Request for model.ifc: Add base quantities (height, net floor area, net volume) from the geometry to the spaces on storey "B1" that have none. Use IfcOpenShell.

First a look at what the model holds.

```python
import ifcopenshell
import ifcopenshell.util.element
import ifcopenshell.util.unit

model = ifcopenshell.open("model.ifc")
print(model.schema)
for unit_type in ("LENGTHUNIT", "AREAUNIT", "VOLUMEUNIT"):
    print(unit_type, ifcopenshell.util.unit.calculate_unit_scale(model, unit_type))
storey = next(s for s in model.by_type("IfcBuildingStorey") if s.Name == "B1")
spaces = [e for e in ifcopenshell.util.element.get_decomposition(storey) if e.is_a("IfcSpace")]
for e in sorted(spaces, key=lambda e: e.id()):
    print(e.id(), e.is_a(), e.Name, list(ifcopenshell.util.element.get_psets(e, qtos_only=True)), sep=" | ")
```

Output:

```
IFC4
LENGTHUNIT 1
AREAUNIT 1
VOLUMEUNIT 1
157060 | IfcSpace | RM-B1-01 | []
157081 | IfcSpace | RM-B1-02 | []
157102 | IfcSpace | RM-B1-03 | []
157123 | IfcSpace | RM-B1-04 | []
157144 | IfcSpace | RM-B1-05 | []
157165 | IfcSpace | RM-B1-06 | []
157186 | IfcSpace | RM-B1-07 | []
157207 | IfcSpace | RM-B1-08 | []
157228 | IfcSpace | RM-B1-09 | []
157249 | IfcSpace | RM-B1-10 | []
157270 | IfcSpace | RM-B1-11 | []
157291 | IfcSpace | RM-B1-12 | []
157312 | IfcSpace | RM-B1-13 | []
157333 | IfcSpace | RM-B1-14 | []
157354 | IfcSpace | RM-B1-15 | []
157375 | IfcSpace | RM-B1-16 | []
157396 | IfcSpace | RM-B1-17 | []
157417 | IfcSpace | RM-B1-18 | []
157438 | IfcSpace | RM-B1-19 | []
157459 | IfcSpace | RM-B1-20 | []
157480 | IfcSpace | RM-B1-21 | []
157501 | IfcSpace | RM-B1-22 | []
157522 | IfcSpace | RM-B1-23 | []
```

```python
import ifcopenshell
import ifcopenshell.api.pset
import ifcopenshell.geom
import ifcopenshell.util.element
import ifcopenshell.util.shape
import ifcopenshell.util.unit

model = ifcopenshell.open("model.ifc")
unit_scale = ifcopenshell.util.unit.calculate_unit_scale(model)
area_scale = ifcopenshell.util.unit.calculate_unit_scale(model, "AREAUNIT")
volume_scale = ifcopenshell.util.unit.calculate_unit_scale(model, "VOLUMEUNIT")
settings = ifcopenshell.geom.settings()

storey = next(s for s in model.by_type("IfcBuildingStorey") if s.Name == "B1")
spaces = [e for e in ifcopenshell.util.element.get_decomposition(storey) if e.is_a("IfcSpace")]

for e in sorted(spaces, key=lambda e: e.id()):
    if ifcopenshell.util.element.get_psets(e, qtos_only=True, should_inherit=False):
        continue
    # Geometry comes back in metres, in the element's own axes.
    shape = ifcopenshell.geom.create_shape(settings, e)
    values = {
        "Height": ifcopenshell.util.shape.get_z(shape.geometry) / unit_scale,
        "NetFloorArea": ifcopenshell.util.shape.get_footprint_area(shape.geometry) / area_scale,
        "NetVolume": ifcopenshell.util.shape.get_volume(shape.geometry) / volume_scale,
    }
    qto = ifcopenshell.api.pset.add_qto(model, product=e, name="Qto_SpaceBaseQuantities")
    ifcopenshell.api.pset.edit_qto(model, qto=qto, properties=values)
    print(e.id(), {k: round(v, 3) for k, v in values.items()})

model.write("model_v2.ifc")
```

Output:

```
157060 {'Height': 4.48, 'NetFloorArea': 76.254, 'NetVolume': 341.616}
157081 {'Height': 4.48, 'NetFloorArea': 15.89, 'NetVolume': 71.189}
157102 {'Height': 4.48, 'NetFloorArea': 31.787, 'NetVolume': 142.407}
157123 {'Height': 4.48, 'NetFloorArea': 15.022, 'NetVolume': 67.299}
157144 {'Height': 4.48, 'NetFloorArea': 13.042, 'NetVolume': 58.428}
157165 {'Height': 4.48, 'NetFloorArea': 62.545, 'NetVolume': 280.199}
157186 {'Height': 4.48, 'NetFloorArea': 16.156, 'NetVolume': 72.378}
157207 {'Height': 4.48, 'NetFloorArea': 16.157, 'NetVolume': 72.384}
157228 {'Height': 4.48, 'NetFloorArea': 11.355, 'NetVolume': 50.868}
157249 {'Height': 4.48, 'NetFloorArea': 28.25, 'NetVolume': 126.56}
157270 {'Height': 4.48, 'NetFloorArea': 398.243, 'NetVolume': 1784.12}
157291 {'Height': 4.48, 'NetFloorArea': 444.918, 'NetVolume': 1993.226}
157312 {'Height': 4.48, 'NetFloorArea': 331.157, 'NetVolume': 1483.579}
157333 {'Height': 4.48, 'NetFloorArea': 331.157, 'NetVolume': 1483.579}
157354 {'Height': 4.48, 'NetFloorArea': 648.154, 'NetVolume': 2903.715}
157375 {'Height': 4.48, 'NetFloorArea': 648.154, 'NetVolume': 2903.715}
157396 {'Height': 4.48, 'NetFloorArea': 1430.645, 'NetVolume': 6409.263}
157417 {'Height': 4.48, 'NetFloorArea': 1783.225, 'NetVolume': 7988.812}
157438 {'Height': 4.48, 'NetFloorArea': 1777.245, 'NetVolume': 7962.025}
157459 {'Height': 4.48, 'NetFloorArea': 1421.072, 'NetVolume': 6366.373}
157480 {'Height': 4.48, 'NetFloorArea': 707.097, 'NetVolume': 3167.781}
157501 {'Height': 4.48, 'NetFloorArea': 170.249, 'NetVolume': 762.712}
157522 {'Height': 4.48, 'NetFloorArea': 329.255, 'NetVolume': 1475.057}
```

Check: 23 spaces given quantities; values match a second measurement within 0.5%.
